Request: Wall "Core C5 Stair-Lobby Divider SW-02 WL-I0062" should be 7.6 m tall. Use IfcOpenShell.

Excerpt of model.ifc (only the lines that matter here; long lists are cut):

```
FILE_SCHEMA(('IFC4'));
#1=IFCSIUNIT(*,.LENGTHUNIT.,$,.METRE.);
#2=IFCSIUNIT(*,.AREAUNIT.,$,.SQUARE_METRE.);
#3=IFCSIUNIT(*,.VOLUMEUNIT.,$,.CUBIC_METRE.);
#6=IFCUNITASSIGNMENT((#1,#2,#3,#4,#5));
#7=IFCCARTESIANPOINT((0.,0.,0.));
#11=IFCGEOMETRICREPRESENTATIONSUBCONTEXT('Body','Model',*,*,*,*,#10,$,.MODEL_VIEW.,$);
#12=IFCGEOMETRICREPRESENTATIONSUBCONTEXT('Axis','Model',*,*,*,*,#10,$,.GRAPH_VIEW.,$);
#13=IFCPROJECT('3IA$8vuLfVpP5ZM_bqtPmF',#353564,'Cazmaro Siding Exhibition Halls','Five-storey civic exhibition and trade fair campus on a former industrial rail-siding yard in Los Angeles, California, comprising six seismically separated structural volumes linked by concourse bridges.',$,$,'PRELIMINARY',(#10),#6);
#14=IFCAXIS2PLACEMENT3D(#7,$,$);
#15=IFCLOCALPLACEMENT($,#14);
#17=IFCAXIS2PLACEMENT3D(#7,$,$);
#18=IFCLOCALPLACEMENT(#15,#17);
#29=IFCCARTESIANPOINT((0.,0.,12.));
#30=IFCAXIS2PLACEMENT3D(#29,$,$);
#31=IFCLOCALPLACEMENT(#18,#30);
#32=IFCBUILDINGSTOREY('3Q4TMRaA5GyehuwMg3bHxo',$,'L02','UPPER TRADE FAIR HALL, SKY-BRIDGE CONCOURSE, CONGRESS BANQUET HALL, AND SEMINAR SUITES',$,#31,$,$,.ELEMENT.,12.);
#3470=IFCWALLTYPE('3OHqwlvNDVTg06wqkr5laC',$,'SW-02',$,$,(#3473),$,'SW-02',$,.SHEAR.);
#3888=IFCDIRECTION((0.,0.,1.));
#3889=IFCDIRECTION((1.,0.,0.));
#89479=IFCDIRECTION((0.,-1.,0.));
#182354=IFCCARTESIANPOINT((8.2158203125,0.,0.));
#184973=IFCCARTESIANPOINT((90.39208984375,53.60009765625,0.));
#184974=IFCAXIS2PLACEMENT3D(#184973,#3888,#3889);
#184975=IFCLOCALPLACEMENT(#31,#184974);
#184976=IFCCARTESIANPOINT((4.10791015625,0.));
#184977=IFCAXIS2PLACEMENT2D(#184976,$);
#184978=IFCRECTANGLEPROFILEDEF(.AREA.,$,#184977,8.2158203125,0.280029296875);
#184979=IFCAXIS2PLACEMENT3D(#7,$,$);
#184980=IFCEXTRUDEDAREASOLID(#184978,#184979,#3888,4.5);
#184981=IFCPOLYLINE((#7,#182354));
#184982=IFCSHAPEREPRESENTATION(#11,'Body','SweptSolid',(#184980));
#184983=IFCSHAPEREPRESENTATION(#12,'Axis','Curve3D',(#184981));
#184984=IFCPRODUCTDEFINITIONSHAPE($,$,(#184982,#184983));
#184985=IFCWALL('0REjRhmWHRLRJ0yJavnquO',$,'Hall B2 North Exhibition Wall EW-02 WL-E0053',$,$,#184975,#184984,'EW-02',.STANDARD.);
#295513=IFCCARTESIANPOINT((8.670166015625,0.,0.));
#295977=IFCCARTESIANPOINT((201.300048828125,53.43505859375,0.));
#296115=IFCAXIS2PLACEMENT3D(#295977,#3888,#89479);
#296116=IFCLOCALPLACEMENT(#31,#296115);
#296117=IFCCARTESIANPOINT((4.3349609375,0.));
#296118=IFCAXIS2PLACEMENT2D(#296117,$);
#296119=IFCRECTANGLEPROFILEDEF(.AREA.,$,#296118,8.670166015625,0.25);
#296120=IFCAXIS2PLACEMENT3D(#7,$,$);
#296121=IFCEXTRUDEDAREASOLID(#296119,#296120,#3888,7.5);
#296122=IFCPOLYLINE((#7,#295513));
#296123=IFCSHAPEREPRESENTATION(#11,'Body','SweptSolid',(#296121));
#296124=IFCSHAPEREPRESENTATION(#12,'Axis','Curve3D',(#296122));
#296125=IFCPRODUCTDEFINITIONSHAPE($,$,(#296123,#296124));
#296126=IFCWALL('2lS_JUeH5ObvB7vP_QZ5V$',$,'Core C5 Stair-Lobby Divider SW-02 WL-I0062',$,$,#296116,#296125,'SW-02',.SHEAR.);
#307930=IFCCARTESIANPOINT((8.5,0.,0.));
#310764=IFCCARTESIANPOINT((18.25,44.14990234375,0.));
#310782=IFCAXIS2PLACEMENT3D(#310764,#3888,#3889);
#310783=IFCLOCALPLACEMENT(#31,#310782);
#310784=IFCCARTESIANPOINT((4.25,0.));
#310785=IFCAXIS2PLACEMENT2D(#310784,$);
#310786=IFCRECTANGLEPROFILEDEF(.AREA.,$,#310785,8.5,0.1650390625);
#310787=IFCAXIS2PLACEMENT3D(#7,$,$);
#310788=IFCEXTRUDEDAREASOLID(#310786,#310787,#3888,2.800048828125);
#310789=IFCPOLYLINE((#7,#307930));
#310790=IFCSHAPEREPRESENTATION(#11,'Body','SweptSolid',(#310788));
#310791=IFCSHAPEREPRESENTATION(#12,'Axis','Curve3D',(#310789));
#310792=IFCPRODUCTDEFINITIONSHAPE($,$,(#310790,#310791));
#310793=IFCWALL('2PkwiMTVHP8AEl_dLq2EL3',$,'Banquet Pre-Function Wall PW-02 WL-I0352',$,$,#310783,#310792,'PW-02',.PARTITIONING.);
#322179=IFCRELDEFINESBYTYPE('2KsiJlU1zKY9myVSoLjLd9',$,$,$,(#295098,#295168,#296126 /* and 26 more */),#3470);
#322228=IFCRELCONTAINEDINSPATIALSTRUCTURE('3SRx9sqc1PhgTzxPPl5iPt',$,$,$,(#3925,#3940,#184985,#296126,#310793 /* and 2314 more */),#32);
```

```python
import ifcopenshell
import ifcopenshell.geom
import ifcopenshell.util.representation
import ifcopenshell.util.shape
import ifcopenshell.util.unit

model = ifcopenshell.open("model.ifc")
unit_scale = ifcopenshell.util.unit.calculate_unit_scale(model)
settings = ifcopenshell.geom.settings()


def volume(element):
    """Net volume in cubic metres, openings subtracted."""
    shape = ifcopenshell.geom.create_shape(settings, element)
    return ifcopenshell.util.shape.get_volume(shape.geometry)


wall = model.by_guid("2lS_JUeH5ObvB7vP_QZ5V$")
before = volume(wall)

body = ifcopenshell.util.representation.get_representation(wall, "Model", "Body")
solid = body.Items[0]
old_height = solid.Depth
solid.Depth = 7.6 / unit_scale
after = volume(wall)

print(f"height {old_height:g} -> {solid.Depth:g}, volume {before:.3f} -> {after:.3f} m3")

model.write("model_v2.ifc")
```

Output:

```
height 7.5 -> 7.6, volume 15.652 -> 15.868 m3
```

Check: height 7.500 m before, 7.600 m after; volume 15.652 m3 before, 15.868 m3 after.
